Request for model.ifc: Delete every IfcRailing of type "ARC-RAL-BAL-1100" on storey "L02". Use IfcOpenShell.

First a look at what the model holds.

```python
import ifcopenshell
import ifcopenshell.util.element

model = ifcopenshell.open("model.ifc")
print(model.schema)
storey = next(s for s in model.by_type("IfcBuildingStorey") if s.Name == "L02")
railings = [e for e in ifcopenshell.util.element.get_decomposition(storey) if e.is_a("IfcRailing")]
seen = {}
for e in railings:
    element_type = ifcopenshell.util.element.get_type(e)
    name = element_type.Name if element_type not in (None, e) else None
    seen[name] = seen.get(name, 0) + 1
for name, count in sorted(seen.items(), key=str):
    print(count, "x", name)
```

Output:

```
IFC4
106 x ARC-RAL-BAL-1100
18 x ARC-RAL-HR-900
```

```python
import ifcopenshell
import ifcopenshell.api.root
import ifcopenshell.util.element

model = ifcopenshell.open("model.ifc")

storey = next(s for s in model.by_type("IfcBuildingStorey") if s.Name == "L02")
railings = [e for e in ifcopenshell.util.element.get_decomposition(storey) if e.is_a("IfcRailing")]
targets = [e for e in railings if (t := ifcopenshell.util.element.get_type(e)) not in (None, e) and t.Name == "ARC-RAL-BAL-1100"]

for e in targets:
    ifcopenshell.api.root.remove_product(model, product=e)
print(len(targets), "removed")

model.write("model_rev.ifc")
```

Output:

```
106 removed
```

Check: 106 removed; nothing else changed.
